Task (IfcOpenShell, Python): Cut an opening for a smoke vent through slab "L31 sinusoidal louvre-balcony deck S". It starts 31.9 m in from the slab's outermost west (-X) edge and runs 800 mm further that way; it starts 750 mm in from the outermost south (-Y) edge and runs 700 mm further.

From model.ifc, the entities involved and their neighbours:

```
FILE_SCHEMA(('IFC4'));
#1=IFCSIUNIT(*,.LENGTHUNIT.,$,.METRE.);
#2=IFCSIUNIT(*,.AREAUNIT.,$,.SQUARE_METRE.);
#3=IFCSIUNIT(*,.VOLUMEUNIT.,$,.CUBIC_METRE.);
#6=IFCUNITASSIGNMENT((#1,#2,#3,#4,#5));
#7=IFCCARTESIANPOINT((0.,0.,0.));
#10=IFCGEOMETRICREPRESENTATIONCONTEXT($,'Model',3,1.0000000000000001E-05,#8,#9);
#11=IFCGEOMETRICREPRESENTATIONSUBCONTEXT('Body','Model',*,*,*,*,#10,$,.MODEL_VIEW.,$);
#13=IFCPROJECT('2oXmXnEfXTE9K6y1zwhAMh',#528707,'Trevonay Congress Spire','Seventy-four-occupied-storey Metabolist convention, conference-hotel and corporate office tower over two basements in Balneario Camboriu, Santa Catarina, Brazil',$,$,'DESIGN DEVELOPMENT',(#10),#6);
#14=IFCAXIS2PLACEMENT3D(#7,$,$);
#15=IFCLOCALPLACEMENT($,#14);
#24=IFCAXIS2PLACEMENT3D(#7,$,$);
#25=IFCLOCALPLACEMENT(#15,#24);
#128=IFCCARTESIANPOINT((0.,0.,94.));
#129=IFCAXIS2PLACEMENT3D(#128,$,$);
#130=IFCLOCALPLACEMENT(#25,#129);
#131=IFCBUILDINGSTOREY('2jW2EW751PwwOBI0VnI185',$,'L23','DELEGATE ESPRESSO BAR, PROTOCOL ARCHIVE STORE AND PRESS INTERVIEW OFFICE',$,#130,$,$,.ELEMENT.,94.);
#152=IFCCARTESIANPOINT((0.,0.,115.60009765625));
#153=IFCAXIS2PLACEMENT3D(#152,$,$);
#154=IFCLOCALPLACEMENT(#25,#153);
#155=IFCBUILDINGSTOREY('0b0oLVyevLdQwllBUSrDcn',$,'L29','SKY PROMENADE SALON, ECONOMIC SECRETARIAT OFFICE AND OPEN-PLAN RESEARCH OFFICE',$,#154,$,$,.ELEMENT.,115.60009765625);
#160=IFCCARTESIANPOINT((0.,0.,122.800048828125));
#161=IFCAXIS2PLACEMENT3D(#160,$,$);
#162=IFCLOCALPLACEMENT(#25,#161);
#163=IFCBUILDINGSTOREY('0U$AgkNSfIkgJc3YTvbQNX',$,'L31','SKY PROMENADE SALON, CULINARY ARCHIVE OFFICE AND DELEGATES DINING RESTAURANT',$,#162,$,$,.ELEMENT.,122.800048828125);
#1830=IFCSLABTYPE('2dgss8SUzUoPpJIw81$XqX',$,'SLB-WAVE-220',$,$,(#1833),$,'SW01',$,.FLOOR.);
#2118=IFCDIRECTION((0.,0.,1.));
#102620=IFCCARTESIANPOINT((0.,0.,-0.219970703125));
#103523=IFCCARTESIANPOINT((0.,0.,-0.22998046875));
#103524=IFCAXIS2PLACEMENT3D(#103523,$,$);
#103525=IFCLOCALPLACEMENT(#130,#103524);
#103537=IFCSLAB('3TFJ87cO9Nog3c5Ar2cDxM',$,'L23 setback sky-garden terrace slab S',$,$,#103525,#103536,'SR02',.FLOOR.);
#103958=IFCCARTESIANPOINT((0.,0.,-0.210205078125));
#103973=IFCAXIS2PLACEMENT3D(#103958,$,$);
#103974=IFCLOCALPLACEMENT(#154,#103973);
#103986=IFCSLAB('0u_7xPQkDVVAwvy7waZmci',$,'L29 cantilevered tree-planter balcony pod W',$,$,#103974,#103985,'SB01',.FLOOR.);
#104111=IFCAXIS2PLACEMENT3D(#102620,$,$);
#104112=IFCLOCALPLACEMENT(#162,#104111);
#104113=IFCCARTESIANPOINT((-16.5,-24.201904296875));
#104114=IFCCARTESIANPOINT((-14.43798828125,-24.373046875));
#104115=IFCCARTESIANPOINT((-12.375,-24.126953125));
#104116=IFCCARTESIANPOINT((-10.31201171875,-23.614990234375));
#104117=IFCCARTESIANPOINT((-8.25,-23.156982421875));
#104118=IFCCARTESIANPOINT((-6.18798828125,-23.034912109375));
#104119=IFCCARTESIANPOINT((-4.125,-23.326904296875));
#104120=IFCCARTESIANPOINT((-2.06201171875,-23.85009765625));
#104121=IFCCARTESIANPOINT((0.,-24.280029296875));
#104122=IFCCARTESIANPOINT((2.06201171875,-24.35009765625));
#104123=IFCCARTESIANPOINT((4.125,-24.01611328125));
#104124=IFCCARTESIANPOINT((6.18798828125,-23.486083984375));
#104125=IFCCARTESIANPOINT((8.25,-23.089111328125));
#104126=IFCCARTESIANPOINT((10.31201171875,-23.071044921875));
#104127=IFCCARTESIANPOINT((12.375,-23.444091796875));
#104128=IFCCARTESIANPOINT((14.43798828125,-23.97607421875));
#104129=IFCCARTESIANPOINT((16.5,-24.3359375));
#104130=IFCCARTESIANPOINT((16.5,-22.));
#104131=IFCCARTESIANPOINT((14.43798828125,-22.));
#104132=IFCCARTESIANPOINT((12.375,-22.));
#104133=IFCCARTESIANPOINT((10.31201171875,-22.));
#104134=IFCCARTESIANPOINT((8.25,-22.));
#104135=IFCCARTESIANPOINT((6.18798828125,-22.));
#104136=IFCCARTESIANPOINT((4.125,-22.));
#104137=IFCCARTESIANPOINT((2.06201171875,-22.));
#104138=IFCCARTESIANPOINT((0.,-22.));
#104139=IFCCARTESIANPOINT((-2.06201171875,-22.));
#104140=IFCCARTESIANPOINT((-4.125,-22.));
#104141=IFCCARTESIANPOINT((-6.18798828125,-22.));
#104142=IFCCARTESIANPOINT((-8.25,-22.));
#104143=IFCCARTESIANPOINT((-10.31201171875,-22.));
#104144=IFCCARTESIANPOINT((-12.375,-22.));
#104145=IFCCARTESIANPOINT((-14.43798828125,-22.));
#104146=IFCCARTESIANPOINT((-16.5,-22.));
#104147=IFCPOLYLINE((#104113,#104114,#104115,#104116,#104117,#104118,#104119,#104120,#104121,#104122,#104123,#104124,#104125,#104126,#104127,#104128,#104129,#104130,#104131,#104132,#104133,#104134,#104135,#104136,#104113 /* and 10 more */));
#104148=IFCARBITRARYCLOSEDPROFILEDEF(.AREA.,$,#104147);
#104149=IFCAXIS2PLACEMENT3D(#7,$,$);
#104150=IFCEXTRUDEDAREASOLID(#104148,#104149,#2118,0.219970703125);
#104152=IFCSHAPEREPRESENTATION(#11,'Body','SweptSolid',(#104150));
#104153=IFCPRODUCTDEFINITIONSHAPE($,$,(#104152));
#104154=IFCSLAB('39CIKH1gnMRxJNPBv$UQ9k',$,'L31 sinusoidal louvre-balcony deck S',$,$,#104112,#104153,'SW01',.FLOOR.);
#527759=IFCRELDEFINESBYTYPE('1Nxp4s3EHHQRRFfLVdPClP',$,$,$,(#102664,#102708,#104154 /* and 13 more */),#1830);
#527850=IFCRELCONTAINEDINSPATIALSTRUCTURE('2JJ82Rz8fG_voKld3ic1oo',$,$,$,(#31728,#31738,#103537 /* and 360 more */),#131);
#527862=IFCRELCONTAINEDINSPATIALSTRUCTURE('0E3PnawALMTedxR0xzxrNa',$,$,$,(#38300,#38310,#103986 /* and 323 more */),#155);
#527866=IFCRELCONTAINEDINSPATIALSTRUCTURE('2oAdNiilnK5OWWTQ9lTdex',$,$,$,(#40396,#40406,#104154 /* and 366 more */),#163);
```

```python
import numpy as np
import ifcopenshell
import ifcopenshell.api.feature
import ifcopenshell.api.geometry
import ifcopenshell.api.root
import ifcopenshell.geom
import ifcopenshell.util.placement
import ifcopenshell.util.representation
import ifcopenshell.util.shape
import ifcopenshell.util.unit

model = ifcopenshell.open("model.ifc")
unit_scale = ifcopenshell.util.unit.calculate_unit_scale(model)
settings = ifcopenshell.geom.settings()


def volume(element):
    """Net volume in cubic metres, openings subtracted."""
    shape = ifcopenshell.geom.create_shape(settings, element)
    return ifcopenshell.util.shape.get_volume(shape.geometry)


slab = model.by_guid("39CIKH1gnMRxJNPBv$UQ9k")
before = volume(slab)

# Extent in the slab's own axes, in metres. The edges named are its -X and -Y sides.
slab_shape = ifcopenshell.geom.create_shape(settings, slab)
vertices = ifcopenshell.util.shape.get_vertices(slab_shape.geometry)
x_min, y_min, bottom = vertices.min(axis=0)
top = vertices[:, 2].max()

opening = ifcopenshell.api.root.create_entity(model, ifc_class="IfcOpeningElement", name="Smoke vent opening", predefined_type="OPENING")
context = ifcopenshell.util.representation.get_context(model, "Model", "Body", "MODEL_VIEW")
width, depth = 0.8, 0.7
outline = [(0.0, 0.0), (width, 0.0), (width, depth), (0.0, depth), (0.0, 0.0)]
# Overshoot both faces by 50 mm so the cut is clean.
shape = ifcopenshell.api.geometry.add_slab_representation(
    model, context=context, depth=top - bottom + 0.1, polyline=outline
)
ifcopenshell.api.geometry.assign_representation(model, product=opening, representation=shape)

matrix = ifcopenshell.util.placement.get_local_placement(slab.ObjectPlacement)
matrix[:, 3] = matrix @ np.append(np.array([x_min + 31.9, y_min + 0.75, bottom - 0.05]) / unit_scale, 1.0)
ifcopenshell.api.geometry.edit_object_placement(model, product=opening, matrix=matrix, is_si=False)
ifcopenshell.api.feature.add_feature(model, feature=opening, element=slab)

after = volume(slab)

print(f"slab volume {before:.3f} -> {after:.3f} m3")

model.write("model_v2.ifc")
```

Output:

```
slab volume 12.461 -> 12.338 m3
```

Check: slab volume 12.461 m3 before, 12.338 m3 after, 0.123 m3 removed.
